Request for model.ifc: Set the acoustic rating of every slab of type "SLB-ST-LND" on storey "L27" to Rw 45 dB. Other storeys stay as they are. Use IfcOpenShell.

First a look at what the model holds.

```python
import ifcopenshell
import ifcopenshell.util.element

model = ifcopenshell.open("model.ifc")
print(model.schema)
storey = next(s for s in model.by_type("IfcBuildingStorey") if s.Name == "L27")
slabs = [e for e in ifcopenshell.util.element.get_decomposition(storey) if e.is_a("IfcSlab")]
seen = {}
for e in slabs:
    element_type = ifcopenshell.util.element.get_type(e)
    key = (element_type.Name if element_type != e and element_type else None, ifcopenshell.util.element.get_pset(e, "Pset_SlabCommon", "AcousticRating"))
    seen[key] = seen.get(key, 0) + 1
for (name, value), count in sorted(seen.items(), key=str):
    print(count, "x", name, "|", value)
```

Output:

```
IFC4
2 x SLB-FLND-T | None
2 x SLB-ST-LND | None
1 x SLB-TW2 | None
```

```python
import ifcopenshell
import ifcopenshell.api.pset
import ifcopenshell.util.element

model = ifcopenshell.open("model.ifc")

storey = next(s for s in model.by_type("IfcBuildingStorey") if s.Name == "L27")
slabs = [e for e in ifcopenshell.util.element.get_decomposition(storey) if e.is_a("IfcSlab")]

count = 0
for e in slabs:
    element_type = ifcopenshell.util.element.get_type(e)
    if element_type in (None, e) or element_type.Name != "SLB-ST-LND":
        continue
    found = ifcopenshell.util.element.get_pset(e, "Pset_SlabCommon", should_inherit=False)
    if found:
        pset = model.by_id(found["id"])
        if len(ifcopenshell.util.element.get_elements_by_pset(pset)) > 1:
            pset = ifcopenshell.api.pset.unshare_pset(model, products=[e], pset=pset)[0]
    else:
        pset = ifcopenshell.api.pset.add_pset(model, product=e, name="Pset_SlabCommon")
    ifcopenshell.api.pset.edit_pset(model, pset=pset, properties={"AcousticRating": "Rw 45 dB"})
    count += 1

print(count, "slabs updated")

model.write("model-out.ifc")
```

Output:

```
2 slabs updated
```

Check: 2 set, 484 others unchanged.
